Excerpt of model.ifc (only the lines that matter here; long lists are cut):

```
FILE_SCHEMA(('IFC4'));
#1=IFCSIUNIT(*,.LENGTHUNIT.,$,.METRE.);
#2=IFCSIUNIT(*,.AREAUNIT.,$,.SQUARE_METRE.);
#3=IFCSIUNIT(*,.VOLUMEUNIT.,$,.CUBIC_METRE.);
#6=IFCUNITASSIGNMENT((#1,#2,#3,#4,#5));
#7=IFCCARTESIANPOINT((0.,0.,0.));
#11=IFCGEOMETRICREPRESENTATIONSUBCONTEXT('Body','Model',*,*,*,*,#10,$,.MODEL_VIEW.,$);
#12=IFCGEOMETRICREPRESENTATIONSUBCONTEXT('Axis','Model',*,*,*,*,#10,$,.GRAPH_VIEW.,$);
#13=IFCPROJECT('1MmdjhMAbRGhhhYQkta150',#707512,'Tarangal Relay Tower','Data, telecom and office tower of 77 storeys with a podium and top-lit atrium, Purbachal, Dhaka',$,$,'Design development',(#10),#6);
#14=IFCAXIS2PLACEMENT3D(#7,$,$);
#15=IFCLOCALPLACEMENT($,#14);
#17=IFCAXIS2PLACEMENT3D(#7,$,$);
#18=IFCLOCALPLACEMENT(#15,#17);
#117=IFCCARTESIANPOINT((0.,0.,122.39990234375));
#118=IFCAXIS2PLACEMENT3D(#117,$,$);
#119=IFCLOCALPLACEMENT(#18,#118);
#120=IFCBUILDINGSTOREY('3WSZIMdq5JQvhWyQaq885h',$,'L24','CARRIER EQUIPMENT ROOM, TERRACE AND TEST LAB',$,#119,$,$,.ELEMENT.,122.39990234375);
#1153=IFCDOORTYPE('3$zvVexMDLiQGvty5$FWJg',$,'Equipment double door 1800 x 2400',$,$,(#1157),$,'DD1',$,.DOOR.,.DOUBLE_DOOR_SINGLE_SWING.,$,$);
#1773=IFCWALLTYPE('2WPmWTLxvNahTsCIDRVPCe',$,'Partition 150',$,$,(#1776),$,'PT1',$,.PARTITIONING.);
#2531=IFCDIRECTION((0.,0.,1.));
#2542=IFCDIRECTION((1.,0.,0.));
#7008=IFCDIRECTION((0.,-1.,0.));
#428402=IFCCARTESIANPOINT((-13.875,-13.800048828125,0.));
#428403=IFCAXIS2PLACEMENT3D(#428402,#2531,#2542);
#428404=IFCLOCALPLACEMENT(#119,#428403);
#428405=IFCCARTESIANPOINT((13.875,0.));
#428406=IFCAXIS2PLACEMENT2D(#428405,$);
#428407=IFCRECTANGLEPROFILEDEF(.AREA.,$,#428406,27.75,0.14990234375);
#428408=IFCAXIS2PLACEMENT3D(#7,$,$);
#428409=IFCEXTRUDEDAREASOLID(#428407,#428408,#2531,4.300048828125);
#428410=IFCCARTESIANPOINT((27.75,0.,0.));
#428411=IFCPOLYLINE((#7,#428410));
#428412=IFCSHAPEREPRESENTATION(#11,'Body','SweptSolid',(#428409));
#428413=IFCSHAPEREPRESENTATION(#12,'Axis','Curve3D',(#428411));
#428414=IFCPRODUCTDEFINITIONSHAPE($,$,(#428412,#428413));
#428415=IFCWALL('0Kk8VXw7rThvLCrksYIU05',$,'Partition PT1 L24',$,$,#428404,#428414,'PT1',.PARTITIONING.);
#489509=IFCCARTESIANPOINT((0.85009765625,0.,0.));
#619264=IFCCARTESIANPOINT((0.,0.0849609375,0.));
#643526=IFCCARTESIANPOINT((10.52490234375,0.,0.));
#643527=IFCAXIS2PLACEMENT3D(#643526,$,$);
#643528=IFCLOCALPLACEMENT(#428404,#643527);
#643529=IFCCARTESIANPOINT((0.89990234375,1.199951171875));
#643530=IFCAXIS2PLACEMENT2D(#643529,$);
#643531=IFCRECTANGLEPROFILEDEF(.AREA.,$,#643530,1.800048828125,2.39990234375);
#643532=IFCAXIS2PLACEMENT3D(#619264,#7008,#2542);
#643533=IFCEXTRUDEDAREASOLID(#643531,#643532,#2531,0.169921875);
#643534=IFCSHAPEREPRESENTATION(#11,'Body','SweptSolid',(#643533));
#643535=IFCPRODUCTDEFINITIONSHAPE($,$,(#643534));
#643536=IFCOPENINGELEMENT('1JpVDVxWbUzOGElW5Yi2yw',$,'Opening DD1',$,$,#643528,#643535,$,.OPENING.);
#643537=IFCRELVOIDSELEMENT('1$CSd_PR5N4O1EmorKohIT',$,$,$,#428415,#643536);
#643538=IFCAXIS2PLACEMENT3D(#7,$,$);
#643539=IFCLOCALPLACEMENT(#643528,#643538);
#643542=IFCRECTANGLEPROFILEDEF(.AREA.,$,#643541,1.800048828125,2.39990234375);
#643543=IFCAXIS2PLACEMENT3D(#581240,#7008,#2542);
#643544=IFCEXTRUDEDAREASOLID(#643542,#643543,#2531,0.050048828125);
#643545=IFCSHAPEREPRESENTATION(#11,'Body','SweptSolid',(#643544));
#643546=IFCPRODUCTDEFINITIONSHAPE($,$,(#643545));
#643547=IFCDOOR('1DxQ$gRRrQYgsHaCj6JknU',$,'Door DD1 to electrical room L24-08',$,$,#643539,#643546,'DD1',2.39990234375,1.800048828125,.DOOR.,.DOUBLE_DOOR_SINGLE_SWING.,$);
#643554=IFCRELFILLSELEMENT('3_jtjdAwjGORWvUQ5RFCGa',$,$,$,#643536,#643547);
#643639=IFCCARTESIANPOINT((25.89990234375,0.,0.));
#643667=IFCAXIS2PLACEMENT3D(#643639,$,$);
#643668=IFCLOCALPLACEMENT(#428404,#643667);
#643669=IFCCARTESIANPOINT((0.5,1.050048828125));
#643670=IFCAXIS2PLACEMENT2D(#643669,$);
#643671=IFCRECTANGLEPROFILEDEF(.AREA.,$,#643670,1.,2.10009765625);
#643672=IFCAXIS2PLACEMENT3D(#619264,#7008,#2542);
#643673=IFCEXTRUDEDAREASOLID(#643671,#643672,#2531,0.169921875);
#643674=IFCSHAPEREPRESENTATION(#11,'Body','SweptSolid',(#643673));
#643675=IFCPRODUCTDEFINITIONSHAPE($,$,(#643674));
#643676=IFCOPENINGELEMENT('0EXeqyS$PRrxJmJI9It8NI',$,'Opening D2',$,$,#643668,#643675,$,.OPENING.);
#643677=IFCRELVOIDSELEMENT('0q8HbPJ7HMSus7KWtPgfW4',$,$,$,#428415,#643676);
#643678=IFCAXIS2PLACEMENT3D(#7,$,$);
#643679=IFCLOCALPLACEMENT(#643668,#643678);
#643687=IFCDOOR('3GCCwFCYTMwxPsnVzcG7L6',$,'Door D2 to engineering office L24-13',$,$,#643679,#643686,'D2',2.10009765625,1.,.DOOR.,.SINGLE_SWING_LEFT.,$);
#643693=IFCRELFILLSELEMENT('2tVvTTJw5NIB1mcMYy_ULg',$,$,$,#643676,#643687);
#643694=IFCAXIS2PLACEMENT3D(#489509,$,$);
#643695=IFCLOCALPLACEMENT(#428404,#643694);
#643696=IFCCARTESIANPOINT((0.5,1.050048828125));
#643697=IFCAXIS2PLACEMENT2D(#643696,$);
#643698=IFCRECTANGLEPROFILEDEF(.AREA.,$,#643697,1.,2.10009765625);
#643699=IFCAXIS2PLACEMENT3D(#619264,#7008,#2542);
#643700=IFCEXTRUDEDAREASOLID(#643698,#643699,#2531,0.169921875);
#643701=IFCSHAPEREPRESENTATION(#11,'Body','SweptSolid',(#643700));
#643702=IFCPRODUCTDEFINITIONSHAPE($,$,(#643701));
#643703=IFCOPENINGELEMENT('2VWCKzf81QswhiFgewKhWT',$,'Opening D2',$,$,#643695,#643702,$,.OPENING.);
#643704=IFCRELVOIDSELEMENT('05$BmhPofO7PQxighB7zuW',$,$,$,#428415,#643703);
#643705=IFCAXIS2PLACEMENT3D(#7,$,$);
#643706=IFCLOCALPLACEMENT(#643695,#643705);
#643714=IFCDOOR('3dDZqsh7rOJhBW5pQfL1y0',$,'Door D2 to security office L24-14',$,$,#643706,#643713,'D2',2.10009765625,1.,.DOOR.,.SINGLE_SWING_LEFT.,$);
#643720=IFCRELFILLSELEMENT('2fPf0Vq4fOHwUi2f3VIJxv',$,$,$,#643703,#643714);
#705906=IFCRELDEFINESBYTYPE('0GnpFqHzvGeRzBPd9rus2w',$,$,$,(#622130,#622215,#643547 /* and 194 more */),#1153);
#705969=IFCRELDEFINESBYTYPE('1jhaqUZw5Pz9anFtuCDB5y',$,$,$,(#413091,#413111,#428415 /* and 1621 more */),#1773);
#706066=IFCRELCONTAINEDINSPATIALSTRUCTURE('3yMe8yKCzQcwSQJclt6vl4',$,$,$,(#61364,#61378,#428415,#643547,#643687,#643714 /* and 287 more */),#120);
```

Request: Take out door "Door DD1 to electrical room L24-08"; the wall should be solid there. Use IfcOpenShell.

```python
import ifcopenshell
import ifcopenshell.api.feature
import ifcopenshell.api.root
import ifcopenshell.geom
import ifcopenshell.util.shape

model = ifcopenshell.open("model.ifc")
settings = ifcopenshell.geom.settings()


def volume(element):
    """Net volume in cubic metres, openings subtracted."""
    shape = ifcopenshell.geom.create_shape(settings, element)
    return ifcopenshell.util.shape.get_volume(shape.geometry)


door = model.by_id(643547)
opening = door.FillsVoids[0].RelatingOpeningElement
wall = opening.VoidsElements[0].RelatingBuildingElement
before = volume(wall)

ifcopenshell.api.root.remove_product(model, product=door)
ifcopenshell.api.feature.remove_feature(model, feature=opening)

after = volume(wall)

print(f"wall volume {before:.3f} -> {after:.3f} m3")

model.write("model_v2.ifc")
```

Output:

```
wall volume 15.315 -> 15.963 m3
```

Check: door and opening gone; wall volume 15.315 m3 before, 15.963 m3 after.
